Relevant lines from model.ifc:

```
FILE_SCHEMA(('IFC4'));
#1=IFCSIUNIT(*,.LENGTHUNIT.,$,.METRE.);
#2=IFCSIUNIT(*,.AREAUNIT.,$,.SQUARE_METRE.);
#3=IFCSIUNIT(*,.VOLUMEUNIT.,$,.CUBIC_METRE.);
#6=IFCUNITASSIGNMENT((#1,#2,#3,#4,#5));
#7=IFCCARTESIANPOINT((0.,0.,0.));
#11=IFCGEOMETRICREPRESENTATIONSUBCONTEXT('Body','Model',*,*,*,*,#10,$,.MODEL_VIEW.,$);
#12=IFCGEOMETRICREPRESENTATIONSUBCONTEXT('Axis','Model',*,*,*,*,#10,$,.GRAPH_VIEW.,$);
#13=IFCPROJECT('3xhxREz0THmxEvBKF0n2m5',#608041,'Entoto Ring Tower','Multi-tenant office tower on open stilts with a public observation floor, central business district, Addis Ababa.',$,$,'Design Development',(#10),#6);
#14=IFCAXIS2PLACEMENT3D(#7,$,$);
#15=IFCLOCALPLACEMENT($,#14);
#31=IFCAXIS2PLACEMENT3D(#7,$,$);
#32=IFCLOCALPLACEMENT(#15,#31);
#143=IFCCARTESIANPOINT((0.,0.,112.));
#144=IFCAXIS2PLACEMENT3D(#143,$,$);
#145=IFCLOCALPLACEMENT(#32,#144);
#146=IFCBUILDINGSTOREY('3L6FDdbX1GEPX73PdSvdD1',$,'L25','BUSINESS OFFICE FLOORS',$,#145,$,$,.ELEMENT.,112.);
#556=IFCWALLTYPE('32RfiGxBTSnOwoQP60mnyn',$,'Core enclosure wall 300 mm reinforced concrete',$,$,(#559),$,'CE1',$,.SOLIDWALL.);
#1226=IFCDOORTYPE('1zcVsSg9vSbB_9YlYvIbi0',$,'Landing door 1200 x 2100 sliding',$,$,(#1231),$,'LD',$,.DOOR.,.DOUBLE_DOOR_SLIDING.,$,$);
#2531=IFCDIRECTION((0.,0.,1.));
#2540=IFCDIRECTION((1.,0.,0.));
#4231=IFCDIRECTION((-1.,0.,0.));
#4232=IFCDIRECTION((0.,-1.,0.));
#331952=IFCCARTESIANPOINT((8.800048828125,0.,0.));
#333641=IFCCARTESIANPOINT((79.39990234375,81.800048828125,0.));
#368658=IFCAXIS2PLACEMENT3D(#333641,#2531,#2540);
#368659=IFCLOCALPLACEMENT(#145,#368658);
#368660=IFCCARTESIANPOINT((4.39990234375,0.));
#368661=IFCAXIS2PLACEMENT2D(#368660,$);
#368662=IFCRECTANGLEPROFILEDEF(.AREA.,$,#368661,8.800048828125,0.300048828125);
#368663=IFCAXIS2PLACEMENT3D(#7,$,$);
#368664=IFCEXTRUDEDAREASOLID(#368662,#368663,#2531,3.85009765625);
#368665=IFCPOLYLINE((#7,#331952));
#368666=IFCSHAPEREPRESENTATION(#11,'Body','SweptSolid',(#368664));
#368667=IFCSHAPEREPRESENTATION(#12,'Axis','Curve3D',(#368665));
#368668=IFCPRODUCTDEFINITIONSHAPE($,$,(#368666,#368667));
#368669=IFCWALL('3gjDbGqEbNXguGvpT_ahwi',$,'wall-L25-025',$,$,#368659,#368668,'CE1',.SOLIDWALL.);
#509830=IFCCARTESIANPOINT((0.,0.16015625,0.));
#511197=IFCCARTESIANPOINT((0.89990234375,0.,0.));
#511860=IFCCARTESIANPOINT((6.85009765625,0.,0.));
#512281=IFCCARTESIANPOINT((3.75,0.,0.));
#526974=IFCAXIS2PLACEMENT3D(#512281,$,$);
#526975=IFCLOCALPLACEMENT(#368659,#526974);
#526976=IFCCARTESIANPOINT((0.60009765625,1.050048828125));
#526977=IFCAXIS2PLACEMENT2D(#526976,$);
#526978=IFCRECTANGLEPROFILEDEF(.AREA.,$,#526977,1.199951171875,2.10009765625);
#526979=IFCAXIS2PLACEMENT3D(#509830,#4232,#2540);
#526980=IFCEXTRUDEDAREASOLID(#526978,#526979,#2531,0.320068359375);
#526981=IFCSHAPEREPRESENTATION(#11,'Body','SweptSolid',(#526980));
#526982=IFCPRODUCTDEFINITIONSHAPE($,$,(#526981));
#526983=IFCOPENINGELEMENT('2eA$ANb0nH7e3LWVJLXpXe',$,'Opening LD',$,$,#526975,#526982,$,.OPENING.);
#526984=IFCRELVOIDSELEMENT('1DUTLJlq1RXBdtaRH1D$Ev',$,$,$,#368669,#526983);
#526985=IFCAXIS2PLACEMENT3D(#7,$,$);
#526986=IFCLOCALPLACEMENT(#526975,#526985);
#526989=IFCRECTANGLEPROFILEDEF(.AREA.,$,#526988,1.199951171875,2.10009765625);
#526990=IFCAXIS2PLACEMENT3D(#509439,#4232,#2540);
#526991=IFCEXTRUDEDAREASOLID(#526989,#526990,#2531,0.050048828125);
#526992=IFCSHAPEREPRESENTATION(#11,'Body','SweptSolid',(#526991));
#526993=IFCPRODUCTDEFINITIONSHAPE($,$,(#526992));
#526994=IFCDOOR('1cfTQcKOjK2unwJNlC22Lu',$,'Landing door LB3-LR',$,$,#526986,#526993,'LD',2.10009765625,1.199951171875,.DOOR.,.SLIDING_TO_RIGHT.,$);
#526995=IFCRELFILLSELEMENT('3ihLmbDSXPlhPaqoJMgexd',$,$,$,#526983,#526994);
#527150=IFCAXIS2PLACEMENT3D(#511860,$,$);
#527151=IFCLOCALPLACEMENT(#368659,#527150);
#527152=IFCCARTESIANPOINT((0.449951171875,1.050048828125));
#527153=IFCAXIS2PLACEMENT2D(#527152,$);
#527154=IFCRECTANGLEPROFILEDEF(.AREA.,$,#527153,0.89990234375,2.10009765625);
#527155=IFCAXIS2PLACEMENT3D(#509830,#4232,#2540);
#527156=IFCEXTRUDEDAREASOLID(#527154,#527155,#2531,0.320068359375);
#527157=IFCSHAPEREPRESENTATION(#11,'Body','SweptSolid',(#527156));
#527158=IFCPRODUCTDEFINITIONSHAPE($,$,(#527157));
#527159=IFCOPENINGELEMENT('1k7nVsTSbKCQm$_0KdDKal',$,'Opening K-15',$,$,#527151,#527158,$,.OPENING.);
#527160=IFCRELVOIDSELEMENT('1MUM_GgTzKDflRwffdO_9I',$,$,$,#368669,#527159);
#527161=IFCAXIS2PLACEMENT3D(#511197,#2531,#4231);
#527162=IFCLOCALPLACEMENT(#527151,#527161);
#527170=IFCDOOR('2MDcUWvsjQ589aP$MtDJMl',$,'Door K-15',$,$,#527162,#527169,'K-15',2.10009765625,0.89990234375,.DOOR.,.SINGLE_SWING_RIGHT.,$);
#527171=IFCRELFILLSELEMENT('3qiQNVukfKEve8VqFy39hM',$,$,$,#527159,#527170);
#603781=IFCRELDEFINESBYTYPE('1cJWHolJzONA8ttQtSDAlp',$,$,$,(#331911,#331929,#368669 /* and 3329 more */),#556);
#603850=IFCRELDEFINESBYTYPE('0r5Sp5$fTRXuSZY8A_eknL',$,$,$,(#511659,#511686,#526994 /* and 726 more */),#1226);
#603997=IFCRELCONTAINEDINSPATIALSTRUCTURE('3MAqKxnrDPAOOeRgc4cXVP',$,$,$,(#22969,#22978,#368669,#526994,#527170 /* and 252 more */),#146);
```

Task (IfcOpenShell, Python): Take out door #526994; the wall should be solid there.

```python
import ifcopenshell
import ifcopenshell.api.feature
import ifcopenshell.api.root
import ifcopenshell.geom
import ifcopenshell.util.shape

model = ifcopenshell.open("model.ifc")
settings = ifcopenshell.geom.settings()


def volume(element):
    """Net volume in cubic metres, openings subtracted."""
    shape = ifcopenshell.geom.create_shape(settings, element)
    return ifcopenshell.util.shape.get_volume(shape.geometry)


door = model.by_id(526994)
opening = door.FillsVoids[0].RelatingOpeningElement
wall = opening.VoidsElements[0].RelatingBuildingElement
before = volume(wall)

ifcopenshell.api.root.remove_product(model, product=door)
ifcopenshell.api.feature.remove_feature(model, feature=opening)

after = volume(wall)

print(f"wall volume {before:.3f} -> {after:.3f} m3")

model.write("model_v2.ifc")
```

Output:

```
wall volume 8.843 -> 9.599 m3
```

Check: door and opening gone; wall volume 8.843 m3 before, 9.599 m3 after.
